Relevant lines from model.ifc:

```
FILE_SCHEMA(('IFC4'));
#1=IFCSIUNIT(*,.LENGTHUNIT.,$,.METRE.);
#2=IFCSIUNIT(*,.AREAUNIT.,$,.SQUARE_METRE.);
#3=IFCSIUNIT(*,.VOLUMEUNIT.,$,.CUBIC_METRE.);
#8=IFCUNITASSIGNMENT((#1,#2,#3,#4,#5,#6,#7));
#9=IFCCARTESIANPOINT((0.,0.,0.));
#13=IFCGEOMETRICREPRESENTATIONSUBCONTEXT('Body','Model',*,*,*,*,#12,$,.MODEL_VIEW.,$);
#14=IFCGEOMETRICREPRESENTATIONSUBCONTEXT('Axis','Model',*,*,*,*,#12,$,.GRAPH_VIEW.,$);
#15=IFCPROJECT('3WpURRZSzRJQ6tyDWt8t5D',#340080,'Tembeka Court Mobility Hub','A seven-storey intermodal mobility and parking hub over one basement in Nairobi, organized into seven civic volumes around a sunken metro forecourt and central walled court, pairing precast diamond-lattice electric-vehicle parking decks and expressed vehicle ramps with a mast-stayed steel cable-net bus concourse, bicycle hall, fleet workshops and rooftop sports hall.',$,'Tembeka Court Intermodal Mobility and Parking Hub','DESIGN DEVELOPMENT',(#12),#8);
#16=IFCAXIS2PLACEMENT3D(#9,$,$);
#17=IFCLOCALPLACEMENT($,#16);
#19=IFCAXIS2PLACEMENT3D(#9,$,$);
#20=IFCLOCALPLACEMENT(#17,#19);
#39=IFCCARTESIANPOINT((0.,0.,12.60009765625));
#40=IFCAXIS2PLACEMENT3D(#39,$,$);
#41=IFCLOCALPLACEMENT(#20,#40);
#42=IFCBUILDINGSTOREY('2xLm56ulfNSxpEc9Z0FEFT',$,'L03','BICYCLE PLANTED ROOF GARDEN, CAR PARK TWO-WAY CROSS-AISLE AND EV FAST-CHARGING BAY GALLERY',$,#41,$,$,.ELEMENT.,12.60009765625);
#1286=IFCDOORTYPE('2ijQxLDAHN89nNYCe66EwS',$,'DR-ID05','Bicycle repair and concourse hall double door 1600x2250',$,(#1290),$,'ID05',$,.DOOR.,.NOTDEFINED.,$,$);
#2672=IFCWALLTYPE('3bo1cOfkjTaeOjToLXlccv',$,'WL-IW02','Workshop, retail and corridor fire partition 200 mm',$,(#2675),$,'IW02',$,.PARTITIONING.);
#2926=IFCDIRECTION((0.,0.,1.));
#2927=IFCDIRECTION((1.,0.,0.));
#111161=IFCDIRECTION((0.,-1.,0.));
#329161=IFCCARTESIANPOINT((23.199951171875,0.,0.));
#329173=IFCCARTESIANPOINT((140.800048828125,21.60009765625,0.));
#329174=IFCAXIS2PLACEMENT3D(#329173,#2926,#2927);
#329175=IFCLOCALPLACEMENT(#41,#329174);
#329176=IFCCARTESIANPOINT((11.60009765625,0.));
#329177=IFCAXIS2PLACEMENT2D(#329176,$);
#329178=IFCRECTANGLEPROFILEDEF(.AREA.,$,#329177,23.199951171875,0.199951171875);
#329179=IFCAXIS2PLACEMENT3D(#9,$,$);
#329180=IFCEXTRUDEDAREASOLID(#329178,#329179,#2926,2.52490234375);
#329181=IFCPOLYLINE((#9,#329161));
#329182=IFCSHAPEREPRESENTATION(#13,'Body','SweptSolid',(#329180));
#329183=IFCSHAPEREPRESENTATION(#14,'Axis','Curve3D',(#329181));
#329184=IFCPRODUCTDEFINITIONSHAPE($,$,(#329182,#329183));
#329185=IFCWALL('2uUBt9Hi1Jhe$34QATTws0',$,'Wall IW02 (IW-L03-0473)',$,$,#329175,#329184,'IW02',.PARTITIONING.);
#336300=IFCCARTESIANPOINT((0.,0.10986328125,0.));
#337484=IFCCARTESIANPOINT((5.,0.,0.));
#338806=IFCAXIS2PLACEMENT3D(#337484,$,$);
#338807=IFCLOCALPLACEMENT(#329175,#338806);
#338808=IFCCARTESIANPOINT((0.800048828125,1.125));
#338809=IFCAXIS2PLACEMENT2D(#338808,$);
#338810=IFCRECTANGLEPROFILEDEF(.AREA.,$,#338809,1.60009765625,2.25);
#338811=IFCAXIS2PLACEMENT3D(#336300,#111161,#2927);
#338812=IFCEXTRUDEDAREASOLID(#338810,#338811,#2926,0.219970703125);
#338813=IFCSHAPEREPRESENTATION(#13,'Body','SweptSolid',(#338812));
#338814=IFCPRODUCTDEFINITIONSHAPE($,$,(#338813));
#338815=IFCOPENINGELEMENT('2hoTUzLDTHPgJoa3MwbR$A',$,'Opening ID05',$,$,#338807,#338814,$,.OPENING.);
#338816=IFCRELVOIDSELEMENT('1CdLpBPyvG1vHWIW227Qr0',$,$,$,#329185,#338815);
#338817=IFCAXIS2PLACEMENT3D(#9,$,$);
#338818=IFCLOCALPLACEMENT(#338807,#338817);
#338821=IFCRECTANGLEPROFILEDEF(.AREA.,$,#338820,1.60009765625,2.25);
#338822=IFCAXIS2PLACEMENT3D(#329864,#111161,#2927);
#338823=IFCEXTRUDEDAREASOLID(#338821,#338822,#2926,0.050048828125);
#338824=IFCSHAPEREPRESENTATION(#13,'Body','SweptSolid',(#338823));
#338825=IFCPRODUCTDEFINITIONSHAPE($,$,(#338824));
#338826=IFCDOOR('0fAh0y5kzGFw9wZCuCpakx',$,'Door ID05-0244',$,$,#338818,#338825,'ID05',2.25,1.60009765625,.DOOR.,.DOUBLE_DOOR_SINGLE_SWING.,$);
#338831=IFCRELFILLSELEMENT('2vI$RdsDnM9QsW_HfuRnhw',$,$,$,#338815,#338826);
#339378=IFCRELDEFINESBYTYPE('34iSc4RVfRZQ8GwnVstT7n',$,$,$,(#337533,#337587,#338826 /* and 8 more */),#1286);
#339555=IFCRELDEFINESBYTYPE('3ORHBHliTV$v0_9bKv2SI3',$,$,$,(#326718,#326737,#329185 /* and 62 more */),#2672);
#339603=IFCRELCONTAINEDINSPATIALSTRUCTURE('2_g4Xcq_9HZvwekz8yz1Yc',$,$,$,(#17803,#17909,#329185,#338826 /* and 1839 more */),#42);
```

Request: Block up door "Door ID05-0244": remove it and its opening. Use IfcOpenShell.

```python
import ifcopenshell
import ifcopenshell.api.feature
import ifcopenshell.api.root
import ifcopenshell.geom
import ifcopenshell.util.shape

model = ifcopenshell.open("model.ifc")
settings = ifcopenshell.geom.settings()


def volume(element):
    """Net volume in cubic metres, openings subtracted."""
    shape = ifcopenshell.geom.create_shape(settings, element)
    return ifcopenshell.util.shape.get_volume(shape.geometry)


door = model.by_id(338826)
opening = door.FillsVoids[0].RelatingOpeningElement
wall = opening.VoidsElements[0].RelatingBuildingElement
before = volume(wall)

ifcopenshell.api.root.remove_product(model, product=door)
ifcopenshell.api.feature.remove_feature(model, feature=opening)

after = volume(wall)

print(f"wall volume {before:.3f} -> {after:.3f} m3")

model.write("model_v2.ifc")
```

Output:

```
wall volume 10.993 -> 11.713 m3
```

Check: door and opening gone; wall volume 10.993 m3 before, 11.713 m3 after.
